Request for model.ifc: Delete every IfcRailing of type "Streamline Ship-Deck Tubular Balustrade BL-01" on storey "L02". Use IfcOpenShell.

First a look at what the model holds.

```python
import ifcopenshell
import ifcopenshell.util.element

model = ifcopenshell.open("model.ifc")
print(model.schema)
storey = next(s for s in model.by_type("IfcBuildingStorey") if s.Name == "L02")
railings = [e for e in ifcopenshell.util.element.get_decomposition(storey) if e.is_a("IfcRailing")]
seen = {}
for e in railings:
    element_type = ifcopenshell.util.element.get_type(e)
    name = element_type.Name if element_type not in (None, e) else None
    seen[name] = seen.get(name, 0) + 1
for name, count in sorted(seen.items(), key=str):
    print(count, "x", name)
```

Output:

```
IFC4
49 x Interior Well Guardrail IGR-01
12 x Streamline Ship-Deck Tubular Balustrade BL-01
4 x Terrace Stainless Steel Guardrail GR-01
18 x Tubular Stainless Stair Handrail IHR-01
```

```python
import ifcopenshell
import ifcopenshell.api.root
import ifcopenshell.util.element

model = ifcopenshell.open("model.ifc")

storey = next(s for s in model.by_type("IfcBuildingStorey") if s.Name == "L02")
railings = [e for e in ifcopenshell.util.element.get_decomposition(storey) if e.is_a("IfcRailing")]
targets = [e for e in railings if (t := ifcopenshell.util.element.get_type(e)) not in (None, e) and t.Name == "Streamline Ship-Deck Tubular Balustrade BL-01"]

for e in targets:
    ifcopenshell.api.root.remove_product(model, product=e)
print(len(targets), "removed")

model.write("model_edited.ifc")
```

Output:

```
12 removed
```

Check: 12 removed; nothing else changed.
